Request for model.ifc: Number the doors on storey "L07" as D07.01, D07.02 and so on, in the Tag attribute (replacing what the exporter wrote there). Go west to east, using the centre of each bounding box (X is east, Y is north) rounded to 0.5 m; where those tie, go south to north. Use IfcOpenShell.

First a look at what the model holds.

```python
import ifcopenshell
import ifcopenshell.util.element
import ifcopenshell.util.placement

model = ifcopenshell.open("model.ifc")
print(model.schema)
storey = next(s for s in model.by_type("IfcBuildingStorey") if s.Name == "L07")
doors = [e for e in ifcopenshell.util.element.get_decomposition(storey) if e.is_a("IfcDoor")]
for e in sorted(doors, key=lambda e: e.id()):
    origin = ifcopenshell.util.placement.get_local_placement(e.ObjectPlacement)[:3, 3]
    print(e.id(), e.Tag, e.Name, origin.round(2) + 0.0, sep=" | ")
```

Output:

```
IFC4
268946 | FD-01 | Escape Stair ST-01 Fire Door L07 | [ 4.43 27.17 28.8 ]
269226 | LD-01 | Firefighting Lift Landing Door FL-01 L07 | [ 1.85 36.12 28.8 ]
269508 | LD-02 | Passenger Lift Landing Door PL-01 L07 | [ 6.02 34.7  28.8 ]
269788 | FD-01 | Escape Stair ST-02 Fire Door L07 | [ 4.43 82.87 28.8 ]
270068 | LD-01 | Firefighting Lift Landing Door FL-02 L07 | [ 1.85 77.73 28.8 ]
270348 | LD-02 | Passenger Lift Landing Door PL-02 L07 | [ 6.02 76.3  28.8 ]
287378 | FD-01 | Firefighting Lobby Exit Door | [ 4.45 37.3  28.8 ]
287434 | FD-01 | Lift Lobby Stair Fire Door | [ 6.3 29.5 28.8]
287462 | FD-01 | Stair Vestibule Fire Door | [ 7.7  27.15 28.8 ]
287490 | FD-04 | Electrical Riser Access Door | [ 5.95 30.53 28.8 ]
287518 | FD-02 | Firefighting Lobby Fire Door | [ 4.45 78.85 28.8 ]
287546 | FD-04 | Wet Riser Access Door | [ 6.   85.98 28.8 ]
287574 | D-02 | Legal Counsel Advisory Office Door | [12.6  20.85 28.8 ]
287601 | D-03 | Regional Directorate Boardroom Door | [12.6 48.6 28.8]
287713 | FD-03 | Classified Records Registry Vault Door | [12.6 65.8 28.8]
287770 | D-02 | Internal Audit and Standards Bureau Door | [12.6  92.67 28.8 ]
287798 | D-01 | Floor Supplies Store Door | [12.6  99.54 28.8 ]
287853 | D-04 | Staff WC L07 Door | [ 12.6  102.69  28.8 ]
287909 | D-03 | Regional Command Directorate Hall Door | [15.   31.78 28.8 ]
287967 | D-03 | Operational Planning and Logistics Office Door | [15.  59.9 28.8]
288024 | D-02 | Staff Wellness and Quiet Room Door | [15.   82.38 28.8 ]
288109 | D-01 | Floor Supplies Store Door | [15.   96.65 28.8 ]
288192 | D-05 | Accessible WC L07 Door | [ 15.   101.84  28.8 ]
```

```python
import ifcopenshell
import ifcopenshell.geom
import ifcopenshell.util.element
import ifcopenshell.util.shape

model = ifcopenshell.open("model.ifc")
settings = ifcopenshell.geom.settings()
settings.set("use-world-coords", True)


def centre(element):
    shape = ifcopenshell.geom.create_shape(settings, element)
    return ifcopenshell.util.shape.get_bbox_centroid(shape.geometry)


storey = next(s for s in model.by_type("IfcBuildingStorey") if s.Name == "L07")
doors = [e for e in ifcopenshell.util.element.get_decomposition(storey) if e.is_a("IfcDoor")]

# Insertion points can sit at a corner or the storey origin, so sort by the geometry (in metres).
centres = {e: centre(e) for e in doors}
doors.sort(key=lambda e: (round(centres[e][0] / 0.5), centres[e][1]))

for i, e in enumerate(doors, start=1):
    number = f"D07.{i:02d}"
    e.Tag = number
    print(e.id(), number)

model.write("model_v2.ifc")
```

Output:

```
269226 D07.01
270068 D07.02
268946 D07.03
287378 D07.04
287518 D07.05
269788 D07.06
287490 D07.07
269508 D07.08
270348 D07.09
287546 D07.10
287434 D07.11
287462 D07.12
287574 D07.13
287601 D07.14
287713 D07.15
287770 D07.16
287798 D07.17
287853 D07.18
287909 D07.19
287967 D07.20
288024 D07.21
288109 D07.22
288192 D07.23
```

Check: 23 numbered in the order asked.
